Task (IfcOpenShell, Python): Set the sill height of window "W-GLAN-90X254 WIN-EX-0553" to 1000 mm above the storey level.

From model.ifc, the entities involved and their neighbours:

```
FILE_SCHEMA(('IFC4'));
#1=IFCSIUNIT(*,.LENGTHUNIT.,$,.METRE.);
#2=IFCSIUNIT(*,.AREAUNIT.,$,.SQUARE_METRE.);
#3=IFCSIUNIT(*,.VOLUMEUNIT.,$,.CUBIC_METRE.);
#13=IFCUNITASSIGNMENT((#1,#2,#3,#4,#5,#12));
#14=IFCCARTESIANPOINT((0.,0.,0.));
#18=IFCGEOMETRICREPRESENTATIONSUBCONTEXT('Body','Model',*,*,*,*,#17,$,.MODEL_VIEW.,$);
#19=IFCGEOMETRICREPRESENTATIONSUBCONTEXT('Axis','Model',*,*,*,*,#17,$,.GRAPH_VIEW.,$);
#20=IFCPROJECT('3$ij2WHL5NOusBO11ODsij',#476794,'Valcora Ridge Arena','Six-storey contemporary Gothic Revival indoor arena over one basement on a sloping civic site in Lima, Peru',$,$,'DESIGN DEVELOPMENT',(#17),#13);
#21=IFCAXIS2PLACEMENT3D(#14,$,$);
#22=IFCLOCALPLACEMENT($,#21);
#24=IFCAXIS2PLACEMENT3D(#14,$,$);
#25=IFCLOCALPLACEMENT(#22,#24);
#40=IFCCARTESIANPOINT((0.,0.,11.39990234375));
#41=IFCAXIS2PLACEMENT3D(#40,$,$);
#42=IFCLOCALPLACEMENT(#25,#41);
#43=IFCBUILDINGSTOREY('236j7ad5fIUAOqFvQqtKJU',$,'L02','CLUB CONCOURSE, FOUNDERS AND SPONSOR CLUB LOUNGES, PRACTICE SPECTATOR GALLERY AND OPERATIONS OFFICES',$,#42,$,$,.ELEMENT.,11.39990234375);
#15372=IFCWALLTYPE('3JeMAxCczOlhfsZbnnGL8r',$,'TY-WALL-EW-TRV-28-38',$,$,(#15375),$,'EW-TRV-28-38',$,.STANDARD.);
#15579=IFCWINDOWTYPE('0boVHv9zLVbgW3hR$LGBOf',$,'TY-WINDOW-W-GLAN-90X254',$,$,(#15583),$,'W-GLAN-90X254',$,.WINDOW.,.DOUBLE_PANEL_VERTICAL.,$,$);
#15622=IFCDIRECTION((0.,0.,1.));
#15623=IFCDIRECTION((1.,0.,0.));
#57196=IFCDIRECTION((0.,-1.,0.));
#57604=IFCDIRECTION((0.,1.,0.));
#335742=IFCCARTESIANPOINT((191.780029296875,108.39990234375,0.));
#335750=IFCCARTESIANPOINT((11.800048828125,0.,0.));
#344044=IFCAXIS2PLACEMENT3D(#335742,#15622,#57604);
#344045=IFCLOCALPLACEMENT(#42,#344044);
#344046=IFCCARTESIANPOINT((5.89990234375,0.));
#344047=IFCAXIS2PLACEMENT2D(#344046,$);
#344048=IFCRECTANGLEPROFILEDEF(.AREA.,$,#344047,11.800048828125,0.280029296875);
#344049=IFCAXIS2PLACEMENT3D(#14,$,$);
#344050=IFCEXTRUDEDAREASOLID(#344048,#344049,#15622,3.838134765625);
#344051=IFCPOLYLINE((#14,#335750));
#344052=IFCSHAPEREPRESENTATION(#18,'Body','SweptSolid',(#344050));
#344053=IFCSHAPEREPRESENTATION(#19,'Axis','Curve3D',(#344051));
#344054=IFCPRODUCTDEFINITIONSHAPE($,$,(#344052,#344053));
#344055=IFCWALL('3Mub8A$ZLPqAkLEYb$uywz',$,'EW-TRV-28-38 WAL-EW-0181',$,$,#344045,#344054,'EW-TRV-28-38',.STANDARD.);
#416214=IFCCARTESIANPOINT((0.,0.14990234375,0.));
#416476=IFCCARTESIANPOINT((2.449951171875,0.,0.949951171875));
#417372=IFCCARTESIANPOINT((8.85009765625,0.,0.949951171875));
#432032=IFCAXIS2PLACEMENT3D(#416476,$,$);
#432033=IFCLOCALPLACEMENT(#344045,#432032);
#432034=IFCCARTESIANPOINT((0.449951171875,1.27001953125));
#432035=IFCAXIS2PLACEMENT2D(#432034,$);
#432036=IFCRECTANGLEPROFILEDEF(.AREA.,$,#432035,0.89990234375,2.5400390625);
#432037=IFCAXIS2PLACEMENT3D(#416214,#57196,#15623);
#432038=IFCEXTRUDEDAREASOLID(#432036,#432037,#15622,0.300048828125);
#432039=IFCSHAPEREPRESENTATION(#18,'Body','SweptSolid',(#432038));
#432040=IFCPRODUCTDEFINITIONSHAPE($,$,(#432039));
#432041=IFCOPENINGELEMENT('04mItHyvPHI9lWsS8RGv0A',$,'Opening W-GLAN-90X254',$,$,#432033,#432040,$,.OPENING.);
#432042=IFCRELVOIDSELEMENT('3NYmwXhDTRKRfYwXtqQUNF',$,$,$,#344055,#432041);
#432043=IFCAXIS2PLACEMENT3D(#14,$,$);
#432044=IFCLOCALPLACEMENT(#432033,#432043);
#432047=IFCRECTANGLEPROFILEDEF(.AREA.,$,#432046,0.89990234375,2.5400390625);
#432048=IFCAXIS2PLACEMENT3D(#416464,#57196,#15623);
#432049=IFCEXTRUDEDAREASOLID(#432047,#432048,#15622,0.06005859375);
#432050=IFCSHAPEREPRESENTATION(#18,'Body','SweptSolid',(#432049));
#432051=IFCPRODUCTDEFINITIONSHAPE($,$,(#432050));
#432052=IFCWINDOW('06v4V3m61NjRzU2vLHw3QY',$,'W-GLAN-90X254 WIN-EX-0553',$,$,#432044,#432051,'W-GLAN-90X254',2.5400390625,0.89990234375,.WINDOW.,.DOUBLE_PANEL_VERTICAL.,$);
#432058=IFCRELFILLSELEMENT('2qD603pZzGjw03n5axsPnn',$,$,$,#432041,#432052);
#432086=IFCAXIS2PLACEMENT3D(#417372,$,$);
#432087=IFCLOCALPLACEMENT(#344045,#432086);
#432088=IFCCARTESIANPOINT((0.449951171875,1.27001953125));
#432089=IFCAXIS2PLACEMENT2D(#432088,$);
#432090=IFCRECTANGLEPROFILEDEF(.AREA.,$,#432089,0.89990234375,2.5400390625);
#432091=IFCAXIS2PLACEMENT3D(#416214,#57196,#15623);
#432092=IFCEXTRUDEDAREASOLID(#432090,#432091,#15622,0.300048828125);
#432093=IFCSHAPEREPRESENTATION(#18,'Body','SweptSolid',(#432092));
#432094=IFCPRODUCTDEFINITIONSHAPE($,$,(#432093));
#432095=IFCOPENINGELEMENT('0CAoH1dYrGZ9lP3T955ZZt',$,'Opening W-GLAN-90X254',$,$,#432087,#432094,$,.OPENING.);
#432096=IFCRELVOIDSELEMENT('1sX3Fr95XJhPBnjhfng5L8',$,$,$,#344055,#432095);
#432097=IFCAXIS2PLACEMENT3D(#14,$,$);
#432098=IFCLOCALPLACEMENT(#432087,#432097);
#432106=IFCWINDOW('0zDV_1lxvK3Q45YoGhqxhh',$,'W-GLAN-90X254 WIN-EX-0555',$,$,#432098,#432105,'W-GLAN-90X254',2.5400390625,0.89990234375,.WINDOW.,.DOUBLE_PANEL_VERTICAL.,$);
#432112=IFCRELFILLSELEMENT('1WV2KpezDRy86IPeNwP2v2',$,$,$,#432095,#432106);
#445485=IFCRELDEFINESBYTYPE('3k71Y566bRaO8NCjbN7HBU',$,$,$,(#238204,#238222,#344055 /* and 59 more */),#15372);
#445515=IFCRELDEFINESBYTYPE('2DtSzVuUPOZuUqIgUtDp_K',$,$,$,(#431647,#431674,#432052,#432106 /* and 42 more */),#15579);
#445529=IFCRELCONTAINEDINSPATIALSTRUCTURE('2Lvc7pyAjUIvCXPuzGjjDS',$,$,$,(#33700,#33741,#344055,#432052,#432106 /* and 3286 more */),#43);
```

```python
import numpy as np
import ifcopenshell
import ifcopenshell.api.geometry
import ifcopenshell.geom
import ifcopenshell.util.element
import ifcopenshell.util.placement
import ifcopenshell.util.shape
import ifcopenshell.util.unit

model = ifcopenshell.open("model.ifc")
unit_scale = ifcopenshell.util.unit.calculate_unit_scale(model)

window = model.by_guid("06v4V3m61NjRzU2vLHw3QY")
opening = window.FillsVoids[0].RelatingOpeningElement
storey = ifcopenshell.util.element.get_container(window, ifc_class="IfcBuildingStorey")
level = ifcopenshell.util.placement.get_local_placement(storey.ObjectPlacement)[2, 3]

# The opening's origin need not be at the sill, so measure its lowest point.
shape = ifcopenshell.geom.create_shape(ifcopenshell.geom.settings(), opening)
bottom = ifcopenshell.util.shape.get_shape_bottom_elevation(shape, shape.geometry) / unit_scale
dz = level + 1 / unit_scale - bottom

shift = np.array([0.0, 0.0, dz])
# The window is placed relative to its opening, so it follows when the opening moves.
matrix = ifcopenshell.util.placement.get_local_placement(opening.ObjectPlacement)
matrix[:3, 3] += shift
ifcopenshell.api.geometry.edit_object_placement(
    model, product=opening, matrix=matrix, is_si=False, should_transform_children=True
)

print(f"moved by {dz * unit_scale:+.3f} m")

model.write("model_v2.ifc")
```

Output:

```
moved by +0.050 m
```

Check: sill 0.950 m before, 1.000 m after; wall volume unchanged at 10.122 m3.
